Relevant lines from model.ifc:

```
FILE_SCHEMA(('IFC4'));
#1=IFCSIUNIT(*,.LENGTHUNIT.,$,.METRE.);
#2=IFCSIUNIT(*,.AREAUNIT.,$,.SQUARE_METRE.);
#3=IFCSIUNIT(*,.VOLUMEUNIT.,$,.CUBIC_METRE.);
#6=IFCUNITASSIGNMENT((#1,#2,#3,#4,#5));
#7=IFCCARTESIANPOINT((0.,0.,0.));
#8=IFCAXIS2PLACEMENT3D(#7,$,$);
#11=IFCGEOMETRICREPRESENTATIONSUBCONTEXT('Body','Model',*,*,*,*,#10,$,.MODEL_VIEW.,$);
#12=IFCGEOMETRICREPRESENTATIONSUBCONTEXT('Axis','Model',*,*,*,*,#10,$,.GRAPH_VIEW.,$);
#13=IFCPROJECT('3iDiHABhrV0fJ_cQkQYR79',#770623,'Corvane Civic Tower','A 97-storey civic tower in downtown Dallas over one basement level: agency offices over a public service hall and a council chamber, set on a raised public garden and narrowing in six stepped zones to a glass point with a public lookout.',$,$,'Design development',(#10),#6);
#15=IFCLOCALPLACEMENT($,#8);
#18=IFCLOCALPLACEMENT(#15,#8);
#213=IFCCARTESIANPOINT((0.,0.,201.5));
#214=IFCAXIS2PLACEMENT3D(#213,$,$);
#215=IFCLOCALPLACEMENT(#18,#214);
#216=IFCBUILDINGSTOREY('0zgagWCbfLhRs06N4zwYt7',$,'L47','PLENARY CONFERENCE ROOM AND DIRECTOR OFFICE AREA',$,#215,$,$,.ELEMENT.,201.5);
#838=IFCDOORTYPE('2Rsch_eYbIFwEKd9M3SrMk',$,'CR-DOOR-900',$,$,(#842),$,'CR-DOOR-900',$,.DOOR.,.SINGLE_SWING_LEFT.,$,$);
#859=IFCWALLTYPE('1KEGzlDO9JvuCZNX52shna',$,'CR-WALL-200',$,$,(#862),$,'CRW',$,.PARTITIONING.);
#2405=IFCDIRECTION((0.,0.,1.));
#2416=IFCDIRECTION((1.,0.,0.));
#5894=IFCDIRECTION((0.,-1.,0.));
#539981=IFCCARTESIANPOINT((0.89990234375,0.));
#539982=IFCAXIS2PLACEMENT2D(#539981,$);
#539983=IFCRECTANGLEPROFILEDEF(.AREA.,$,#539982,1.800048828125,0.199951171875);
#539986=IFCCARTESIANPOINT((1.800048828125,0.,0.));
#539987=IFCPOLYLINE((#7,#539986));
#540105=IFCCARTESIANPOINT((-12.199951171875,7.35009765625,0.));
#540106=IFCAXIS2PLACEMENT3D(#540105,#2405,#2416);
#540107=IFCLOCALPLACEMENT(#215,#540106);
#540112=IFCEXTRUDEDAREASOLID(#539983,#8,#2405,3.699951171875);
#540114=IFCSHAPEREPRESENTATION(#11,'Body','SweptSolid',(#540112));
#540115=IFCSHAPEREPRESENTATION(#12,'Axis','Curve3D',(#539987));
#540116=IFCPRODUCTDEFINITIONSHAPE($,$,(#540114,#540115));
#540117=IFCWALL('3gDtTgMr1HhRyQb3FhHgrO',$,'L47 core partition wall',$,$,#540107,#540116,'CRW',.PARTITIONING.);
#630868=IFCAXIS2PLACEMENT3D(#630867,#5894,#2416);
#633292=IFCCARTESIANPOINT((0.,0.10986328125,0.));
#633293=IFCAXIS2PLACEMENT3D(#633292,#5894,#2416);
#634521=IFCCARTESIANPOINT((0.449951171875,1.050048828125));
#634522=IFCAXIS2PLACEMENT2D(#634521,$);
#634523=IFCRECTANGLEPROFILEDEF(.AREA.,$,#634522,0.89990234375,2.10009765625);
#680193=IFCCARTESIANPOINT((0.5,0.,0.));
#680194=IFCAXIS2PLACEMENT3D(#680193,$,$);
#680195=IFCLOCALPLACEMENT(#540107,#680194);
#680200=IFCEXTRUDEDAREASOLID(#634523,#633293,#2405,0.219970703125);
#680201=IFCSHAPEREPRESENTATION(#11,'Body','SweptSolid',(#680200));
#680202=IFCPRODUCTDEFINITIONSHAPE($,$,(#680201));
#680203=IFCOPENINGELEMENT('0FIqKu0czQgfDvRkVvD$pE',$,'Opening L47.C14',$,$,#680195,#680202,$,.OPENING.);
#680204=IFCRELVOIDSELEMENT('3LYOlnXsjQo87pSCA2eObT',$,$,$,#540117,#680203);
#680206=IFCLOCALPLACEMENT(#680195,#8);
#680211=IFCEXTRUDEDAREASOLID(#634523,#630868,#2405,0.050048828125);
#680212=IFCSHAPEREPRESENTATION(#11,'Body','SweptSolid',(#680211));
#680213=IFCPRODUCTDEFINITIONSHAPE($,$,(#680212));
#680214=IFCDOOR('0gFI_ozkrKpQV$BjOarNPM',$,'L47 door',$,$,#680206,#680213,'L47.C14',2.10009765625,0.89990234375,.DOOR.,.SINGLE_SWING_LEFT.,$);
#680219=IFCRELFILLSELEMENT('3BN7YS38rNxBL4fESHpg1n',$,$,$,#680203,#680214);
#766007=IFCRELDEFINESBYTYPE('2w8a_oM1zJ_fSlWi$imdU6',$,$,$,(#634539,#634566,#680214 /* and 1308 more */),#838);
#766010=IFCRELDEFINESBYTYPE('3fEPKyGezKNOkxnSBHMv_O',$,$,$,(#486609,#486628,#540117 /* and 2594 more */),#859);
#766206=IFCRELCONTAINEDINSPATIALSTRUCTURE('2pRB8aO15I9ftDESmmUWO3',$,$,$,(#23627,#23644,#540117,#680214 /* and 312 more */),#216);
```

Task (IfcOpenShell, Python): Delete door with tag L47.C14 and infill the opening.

```python
import ifcopenshell
import ifcopenshell.api.feature
import ifcopenshell.api.root
import ifcopenshell.geom
import ifcopenshell.util.shape

model = ifcopenshell.open("model.ifc")
settings = ifcopenshell.geom.settings()


def volume(element):
    """Net volume in cubic metres, openings subtracted."""
    shape = ifcopenshell.geom.create_shape(settings, element)
    return ifcopenshell.util.shape.get_volume(shape.geometry)


door = model.by_guid("0gFI_ozkrKpQV$BjOarNPM")
opening = door.FillsVoids[0].RelatingOpeningElement
wall = opening.VoidsElements[0].RelatingBuildingElement
before = volume(wall)

ifcopenshell.api.root.remove_product(model, product=door)
ifcopenshell.api.feature.remove_feature(model, feature=opening)

after = volume(wall)

print(f"wall volume {before:.3f} -> {after:.3f} m3")

model.write("model-out.ifc")
```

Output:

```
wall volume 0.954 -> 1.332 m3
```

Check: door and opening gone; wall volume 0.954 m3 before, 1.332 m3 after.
